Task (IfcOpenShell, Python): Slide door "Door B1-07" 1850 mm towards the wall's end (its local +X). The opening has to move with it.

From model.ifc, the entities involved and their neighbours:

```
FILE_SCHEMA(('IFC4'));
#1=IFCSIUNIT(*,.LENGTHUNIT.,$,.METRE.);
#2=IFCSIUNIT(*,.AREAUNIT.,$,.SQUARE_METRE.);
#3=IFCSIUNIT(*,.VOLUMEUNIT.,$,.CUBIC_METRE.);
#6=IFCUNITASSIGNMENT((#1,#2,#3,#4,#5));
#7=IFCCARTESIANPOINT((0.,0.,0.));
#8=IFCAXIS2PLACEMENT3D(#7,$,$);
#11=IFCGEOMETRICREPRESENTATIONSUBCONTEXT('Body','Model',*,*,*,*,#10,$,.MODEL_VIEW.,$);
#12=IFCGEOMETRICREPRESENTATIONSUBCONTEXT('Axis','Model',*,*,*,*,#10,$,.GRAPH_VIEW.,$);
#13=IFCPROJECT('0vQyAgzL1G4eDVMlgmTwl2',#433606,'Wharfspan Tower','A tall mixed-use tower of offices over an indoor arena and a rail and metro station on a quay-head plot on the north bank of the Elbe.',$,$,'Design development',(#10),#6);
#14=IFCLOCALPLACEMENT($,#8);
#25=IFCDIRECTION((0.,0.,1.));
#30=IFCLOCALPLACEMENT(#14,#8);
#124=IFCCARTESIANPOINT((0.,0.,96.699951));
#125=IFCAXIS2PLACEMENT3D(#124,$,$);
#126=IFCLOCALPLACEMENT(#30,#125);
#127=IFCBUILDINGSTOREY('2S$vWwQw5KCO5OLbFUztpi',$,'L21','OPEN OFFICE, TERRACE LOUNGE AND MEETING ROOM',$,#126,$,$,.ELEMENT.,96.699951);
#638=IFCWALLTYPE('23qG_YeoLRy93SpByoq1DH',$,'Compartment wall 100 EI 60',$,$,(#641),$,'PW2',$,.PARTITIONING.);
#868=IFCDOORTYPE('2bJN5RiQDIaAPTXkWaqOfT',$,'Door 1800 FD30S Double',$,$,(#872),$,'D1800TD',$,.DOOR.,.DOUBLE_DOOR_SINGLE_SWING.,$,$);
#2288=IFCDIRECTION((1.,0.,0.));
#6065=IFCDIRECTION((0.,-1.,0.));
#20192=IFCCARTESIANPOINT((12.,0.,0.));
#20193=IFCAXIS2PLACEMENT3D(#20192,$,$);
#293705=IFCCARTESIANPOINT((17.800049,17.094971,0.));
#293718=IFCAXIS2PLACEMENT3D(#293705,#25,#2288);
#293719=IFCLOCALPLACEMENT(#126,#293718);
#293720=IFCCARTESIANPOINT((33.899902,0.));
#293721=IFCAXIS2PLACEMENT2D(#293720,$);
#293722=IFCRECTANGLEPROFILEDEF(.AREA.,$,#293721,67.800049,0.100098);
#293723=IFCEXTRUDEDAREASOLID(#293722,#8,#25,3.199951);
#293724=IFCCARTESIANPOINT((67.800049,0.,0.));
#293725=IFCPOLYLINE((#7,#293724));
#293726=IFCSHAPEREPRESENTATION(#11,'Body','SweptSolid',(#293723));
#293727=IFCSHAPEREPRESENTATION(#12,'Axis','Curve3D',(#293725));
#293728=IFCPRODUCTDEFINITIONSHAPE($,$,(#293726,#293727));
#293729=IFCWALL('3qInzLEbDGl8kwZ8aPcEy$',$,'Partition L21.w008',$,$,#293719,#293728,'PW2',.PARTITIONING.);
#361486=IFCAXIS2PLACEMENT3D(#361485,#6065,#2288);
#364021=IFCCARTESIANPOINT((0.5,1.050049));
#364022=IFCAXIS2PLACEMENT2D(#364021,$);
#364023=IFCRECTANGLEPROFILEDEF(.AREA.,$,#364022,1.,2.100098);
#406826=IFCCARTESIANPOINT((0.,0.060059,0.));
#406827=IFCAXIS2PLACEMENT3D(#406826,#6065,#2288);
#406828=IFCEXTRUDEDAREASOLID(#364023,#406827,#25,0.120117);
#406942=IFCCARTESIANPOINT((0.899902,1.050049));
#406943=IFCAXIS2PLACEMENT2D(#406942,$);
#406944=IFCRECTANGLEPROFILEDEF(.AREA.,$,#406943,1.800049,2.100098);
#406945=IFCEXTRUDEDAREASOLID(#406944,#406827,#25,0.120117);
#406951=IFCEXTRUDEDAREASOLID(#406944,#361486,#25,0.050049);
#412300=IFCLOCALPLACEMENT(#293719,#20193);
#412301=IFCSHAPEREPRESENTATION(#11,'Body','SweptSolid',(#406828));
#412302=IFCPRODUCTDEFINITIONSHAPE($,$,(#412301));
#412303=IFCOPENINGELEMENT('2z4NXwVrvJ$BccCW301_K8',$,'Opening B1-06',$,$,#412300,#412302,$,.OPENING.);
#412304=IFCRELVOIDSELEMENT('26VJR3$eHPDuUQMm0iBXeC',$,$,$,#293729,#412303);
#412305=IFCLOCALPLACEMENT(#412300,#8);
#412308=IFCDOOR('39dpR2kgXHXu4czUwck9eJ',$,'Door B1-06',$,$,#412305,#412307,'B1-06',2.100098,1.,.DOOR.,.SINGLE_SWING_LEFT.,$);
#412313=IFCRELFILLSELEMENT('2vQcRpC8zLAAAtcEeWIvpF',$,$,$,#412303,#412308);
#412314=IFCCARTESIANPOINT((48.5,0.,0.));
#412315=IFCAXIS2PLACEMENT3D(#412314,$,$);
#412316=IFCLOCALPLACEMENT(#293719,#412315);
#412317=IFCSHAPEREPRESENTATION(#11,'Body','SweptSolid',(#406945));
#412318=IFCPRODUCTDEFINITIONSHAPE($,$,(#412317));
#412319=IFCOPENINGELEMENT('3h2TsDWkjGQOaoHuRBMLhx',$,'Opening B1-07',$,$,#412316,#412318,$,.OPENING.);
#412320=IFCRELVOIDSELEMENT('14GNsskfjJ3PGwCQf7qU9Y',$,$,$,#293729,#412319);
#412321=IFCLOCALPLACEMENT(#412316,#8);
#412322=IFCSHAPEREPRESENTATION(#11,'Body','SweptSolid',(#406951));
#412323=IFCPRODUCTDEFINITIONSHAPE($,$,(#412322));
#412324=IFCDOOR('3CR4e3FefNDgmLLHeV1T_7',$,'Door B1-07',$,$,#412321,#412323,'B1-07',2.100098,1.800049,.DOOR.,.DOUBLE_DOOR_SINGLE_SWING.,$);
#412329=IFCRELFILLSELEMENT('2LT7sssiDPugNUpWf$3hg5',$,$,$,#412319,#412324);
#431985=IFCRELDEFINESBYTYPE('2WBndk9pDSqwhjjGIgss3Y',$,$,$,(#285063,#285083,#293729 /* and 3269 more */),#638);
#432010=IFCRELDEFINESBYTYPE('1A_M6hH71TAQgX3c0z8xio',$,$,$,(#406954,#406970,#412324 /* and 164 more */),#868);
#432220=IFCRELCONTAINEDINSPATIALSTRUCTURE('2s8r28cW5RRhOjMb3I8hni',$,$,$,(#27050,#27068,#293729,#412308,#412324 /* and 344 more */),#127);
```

```python
import ifcopenshell
import ifcopenshell.api.geometry
import ifcopenshell.util.placement
import ifcopenshell.util.unit

model = ifcopenshell.open("model.ifc")
unit_scale = ifcopenshell.util.unit.calculate_unit_scale(model)

door = model.by_guid("3CR4e3FefNDgmLLHeV1T_7")
opening = door.FillsVoids[0].RelatingOpeningElement
wall = opening.VoidsElements[0].RelatingBuildingElement

wall_matrix = ifcopenshell.util.placement.get_local_placement(wall.ObjectPlacement)
shift = wall_matrix[:3, 0] * 1.85 / unit_scale
before = ifcopenshell.util.placement.get_local_placement(door.ObjectPlacement)[:3, 3].copy()

# The door is placed relative to its opening, so it follows when the opening moves.
matrix = ifcopenshell.util.placement.get_local_placement(opening.ObjectPlacement)
matrix[:3, 3] += shift
ifcopenshell.api.geometry.edit_object_placement(
    model, product=opening, matrix=matrix, is_si=False, should_transform_children=True
)

after = ifcopenshell.util.placement.get_local_placement(door.ObjectPlacement)[:3, 3]
print("door moved by", (after - before).round(3) + 0.0)

model.write("model_rev.ifc")
```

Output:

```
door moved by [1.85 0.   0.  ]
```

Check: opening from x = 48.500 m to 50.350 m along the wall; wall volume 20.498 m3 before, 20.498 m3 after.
